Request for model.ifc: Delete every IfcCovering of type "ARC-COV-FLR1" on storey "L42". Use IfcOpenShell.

First a look at what the model holds.

```python
import ifcopenshell
import ifcopenshell.util.element

model = ifcopenshell.open("model.ifc")
print(model.schema)
storey = next(s for s in model.by_type("IfcBuildingStorey") if s.Name == "L42")
coverings = [e for e in ifcopenshell.util.element.get_decomposition(storey) if e.is_a("IfcCovering")]
seen = {}
for e in coverings:
    element_type = ifcopenshell.util.element.get_type(e)
    name = element_type.Name if element_type not in (None, e) else None
    seen[name] = seen.get(name, 0) + 1
for name, count in sorted(seen.items(), key=str):
    print(count, "x", name)
```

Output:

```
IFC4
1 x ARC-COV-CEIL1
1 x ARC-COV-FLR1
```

```python
import ifcopenshell
import ifcopenshell.api.root
import ifcopenshell.util.element

model = ifcopenshell.open("model.ifc")

storey = next(s for s in model.by_type("IfcBuildingStorey") if s.Name == "L42")
coverings = [e for e in ifcopenshell.util.element.get_decomposition(storey) if e.is_a("IfcCovering")]
targets = [e for e in coverings if (t := ifcopenshell.util.element.get_type(e)) not in (None, e) and t.Name == "ARC-COV-FLR1"]

for e in targets:
    ifcopenshell.api.root.remove_product(model, product=e)
print(len(targets), "removed")

model.write("model-out.ifc")
```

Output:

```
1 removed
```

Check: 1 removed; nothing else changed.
